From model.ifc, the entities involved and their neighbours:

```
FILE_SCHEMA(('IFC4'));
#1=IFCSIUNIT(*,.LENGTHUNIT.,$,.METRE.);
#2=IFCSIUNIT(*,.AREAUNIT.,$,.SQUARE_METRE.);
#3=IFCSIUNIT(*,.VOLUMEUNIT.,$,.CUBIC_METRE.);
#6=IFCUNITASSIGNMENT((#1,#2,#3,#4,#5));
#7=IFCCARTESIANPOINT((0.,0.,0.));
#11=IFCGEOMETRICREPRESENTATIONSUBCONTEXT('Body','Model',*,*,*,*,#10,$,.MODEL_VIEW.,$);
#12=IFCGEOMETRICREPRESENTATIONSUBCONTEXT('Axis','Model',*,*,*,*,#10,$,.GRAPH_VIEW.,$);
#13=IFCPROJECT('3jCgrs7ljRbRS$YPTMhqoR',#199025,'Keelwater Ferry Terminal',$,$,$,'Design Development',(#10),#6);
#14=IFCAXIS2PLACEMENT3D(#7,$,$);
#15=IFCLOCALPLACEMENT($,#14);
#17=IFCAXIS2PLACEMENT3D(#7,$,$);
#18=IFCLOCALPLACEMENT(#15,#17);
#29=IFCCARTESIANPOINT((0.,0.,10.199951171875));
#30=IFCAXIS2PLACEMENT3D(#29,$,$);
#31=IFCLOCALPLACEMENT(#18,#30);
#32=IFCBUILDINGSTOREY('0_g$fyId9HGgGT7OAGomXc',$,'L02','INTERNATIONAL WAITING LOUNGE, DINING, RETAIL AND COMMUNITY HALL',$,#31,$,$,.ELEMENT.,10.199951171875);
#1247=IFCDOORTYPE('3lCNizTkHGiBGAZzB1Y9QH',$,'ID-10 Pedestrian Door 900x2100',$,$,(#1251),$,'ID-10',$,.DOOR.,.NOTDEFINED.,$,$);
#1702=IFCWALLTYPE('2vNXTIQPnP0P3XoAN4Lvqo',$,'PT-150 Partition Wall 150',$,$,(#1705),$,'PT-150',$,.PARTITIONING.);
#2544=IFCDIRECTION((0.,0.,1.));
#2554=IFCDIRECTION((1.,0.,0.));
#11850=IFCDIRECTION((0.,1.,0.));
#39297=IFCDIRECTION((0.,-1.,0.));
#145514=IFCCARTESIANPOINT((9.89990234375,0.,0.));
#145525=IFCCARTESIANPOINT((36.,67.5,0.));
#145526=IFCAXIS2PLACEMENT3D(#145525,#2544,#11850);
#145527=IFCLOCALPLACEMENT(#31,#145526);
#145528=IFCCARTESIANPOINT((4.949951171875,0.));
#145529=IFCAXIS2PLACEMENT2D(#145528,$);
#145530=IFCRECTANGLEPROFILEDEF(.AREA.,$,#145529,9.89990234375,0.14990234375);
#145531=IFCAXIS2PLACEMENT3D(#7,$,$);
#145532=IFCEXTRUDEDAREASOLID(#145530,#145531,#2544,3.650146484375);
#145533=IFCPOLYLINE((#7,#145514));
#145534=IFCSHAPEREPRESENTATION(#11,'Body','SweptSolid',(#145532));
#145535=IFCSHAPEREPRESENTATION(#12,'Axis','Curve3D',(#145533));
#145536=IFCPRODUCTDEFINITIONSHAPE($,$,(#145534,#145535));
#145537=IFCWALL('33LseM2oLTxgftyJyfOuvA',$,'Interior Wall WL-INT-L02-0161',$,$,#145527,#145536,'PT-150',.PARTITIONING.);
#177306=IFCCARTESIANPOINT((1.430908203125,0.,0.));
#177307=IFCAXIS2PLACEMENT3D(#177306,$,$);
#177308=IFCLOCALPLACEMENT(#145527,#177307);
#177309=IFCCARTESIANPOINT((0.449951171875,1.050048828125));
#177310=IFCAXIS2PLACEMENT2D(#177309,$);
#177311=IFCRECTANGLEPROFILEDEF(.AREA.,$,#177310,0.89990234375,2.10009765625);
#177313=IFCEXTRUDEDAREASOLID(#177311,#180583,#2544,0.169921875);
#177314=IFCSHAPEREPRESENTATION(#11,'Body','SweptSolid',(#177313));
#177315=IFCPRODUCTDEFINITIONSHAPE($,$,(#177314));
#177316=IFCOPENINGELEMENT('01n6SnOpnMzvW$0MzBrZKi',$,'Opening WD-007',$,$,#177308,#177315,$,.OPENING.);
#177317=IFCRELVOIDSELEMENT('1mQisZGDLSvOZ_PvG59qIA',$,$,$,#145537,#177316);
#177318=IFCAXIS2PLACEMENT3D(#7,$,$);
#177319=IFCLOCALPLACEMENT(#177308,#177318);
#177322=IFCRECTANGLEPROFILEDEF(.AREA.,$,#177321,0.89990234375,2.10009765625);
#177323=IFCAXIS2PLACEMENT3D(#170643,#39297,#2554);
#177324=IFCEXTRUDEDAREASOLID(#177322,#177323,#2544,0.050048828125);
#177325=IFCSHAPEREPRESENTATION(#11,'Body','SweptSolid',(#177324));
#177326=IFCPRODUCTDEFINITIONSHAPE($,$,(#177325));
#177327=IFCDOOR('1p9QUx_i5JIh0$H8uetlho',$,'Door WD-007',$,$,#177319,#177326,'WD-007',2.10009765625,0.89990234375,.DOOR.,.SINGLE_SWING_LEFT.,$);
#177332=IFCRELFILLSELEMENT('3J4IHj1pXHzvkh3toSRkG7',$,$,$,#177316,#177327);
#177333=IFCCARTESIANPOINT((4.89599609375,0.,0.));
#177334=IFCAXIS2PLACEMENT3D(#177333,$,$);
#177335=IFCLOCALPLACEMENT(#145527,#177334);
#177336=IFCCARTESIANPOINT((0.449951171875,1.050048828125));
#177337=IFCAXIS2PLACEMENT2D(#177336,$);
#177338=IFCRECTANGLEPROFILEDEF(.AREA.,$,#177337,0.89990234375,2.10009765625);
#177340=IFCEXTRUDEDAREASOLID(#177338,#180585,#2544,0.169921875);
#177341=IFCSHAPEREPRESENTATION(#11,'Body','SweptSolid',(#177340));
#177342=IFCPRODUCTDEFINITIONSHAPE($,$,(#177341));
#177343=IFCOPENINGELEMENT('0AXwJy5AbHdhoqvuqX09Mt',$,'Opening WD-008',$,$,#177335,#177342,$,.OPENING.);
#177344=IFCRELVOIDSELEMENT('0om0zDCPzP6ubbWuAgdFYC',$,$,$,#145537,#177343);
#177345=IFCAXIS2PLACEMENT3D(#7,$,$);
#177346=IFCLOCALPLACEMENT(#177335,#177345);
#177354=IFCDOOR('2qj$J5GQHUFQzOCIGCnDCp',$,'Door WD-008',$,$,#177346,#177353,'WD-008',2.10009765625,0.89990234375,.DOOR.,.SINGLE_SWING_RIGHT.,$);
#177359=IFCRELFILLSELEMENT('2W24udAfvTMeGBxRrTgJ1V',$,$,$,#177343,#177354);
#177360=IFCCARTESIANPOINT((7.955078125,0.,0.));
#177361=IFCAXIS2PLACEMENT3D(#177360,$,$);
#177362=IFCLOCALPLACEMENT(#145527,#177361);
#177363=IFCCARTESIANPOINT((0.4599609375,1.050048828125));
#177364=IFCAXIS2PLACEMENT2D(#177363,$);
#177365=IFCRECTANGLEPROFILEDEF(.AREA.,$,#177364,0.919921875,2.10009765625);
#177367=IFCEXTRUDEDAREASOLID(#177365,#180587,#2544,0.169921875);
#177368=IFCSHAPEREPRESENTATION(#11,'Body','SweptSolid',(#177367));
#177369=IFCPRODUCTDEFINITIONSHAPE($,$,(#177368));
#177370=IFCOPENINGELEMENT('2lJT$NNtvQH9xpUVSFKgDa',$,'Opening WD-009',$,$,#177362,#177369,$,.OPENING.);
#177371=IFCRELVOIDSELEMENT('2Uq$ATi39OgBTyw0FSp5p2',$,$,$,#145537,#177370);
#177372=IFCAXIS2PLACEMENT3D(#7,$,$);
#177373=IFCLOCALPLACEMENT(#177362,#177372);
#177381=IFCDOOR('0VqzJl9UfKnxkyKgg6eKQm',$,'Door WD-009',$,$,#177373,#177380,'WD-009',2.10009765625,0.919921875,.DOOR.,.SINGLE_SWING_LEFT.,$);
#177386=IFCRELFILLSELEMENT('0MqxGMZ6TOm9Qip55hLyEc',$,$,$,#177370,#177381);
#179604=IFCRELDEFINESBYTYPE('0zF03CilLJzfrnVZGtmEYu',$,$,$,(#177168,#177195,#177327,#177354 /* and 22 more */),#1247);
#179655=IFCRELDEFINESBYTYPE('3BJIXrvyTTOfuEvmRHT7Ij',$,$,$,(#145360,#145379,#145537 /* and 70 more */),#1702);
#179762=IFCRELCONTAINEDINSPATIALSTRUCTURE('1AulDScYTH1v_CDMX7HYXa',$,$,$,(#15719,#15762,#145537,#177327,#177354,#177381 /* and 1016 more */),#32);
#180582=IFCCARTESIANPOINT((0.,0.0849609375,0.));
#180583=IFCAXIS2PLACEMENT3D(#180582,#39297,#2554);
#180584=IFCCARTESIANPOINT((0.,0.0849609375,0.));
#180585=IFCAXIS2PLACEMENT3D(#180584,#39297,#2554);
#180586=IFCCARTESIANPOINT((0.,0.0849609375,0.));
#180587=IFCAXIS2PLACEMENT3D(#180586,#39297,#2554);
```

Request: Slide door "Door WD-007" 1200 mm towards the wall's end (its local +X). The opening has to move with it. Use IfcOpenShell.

```python
import ifcopenshell
import ifcopenshell.api.geometry
import ifcopenshell.util.placement
import ifcopenshell.util.unit

model = ifcopenshell.open("model.ifc")
unit_scale = ifcopenshell.util.unit.calculate_unit_scale(model)

door = model.by_guid("1p9QUx_i5JIh0$H8uetlho")
opening = door.FillsVoids[0].RelatingOpeningElement
wall = opening.VoidsElements[0].RelatingBuildingElement

wall_matrix = ifcopenshell.util.placement.get_local_placement(wall.ObjectPlacement)
shift = wall_matrix[:3, 0] * 1.2 / unit_scale
before = ifcopenshell.util.placement.get_local_placement(door.ObjectPlacement)[:3, 3].copy()

# The door is placed relative to its opening, so it follows when the opening moves.
matrix = ifcopenshell.util.placement.get_local_placement(opening.ObjectPlacement)
matrix[:3, 3] += shift
ifcopenshell.api.geometry.edit_object_placement(
    model, product=opening, matrix=matrix, is_si=False, should_transform_children=True
)

after = ifcopenshell.util.placement.get_local_placement(door.ObjectPlacement)[:3, 3]
print("door moved by", (after - before).round(3) + 0.0)

model.write("model_rev.ifc")
```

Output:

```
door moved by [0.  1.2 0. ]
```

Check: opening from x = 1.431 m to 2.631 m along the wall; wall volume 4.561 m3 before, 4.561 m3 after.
